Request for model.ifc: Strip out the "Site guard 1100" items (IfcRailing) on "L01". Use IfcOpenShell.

First a look at what the model holds.

```python
import ifcopenshell
import ifcopenshell.util.element

model = ifcopenshell.open("model.ifc")
print(model.schema)
storey = next(s for s in model.by_type("IfcBuildingStorey") if s.Name == "L01")
railings = [e for e in ifcopenshell.util.element.get_decomposition(storey) if e.is_a("IfcRailing")]
seen = {}
for e in railings:
    element_type = ifcopenshell.util.element.get_type(e)
    name = element_type.Name if element_type not in (None, e) else None
    seen[name] = seen.get(name, 0) + 1
for name, count in sorted(seen.items(), key=str):
    print(count, "x", name)
```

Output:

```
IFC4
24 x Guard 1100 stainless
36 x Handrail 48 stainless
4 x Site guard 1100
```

```python
import ifcopenshell
import ifcopenshell.api.root
import ifcopenshell.util.element

model = ifcopenshell.open("model.ifc")

storey = next(s for s in model.by_type("IfcBuildingStorey") if s.Name == "L01")
railings = [e for e in ifcopenshell.util.element.get_decomposition(storey) if e.is_a("IfcRailing")]
targets = [e for e in railings if (t := ifcopenshell.util.element.get_type(e)) not in (None, e) and t.Name == "Site guard 1100"]

for e in targets:
    ifcopenshell.api.root.remove_product(model, product=e)
print(len(targets), "removed")

model.write("model_v2.ifc")
```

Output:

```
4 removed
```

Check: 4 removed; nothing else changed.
